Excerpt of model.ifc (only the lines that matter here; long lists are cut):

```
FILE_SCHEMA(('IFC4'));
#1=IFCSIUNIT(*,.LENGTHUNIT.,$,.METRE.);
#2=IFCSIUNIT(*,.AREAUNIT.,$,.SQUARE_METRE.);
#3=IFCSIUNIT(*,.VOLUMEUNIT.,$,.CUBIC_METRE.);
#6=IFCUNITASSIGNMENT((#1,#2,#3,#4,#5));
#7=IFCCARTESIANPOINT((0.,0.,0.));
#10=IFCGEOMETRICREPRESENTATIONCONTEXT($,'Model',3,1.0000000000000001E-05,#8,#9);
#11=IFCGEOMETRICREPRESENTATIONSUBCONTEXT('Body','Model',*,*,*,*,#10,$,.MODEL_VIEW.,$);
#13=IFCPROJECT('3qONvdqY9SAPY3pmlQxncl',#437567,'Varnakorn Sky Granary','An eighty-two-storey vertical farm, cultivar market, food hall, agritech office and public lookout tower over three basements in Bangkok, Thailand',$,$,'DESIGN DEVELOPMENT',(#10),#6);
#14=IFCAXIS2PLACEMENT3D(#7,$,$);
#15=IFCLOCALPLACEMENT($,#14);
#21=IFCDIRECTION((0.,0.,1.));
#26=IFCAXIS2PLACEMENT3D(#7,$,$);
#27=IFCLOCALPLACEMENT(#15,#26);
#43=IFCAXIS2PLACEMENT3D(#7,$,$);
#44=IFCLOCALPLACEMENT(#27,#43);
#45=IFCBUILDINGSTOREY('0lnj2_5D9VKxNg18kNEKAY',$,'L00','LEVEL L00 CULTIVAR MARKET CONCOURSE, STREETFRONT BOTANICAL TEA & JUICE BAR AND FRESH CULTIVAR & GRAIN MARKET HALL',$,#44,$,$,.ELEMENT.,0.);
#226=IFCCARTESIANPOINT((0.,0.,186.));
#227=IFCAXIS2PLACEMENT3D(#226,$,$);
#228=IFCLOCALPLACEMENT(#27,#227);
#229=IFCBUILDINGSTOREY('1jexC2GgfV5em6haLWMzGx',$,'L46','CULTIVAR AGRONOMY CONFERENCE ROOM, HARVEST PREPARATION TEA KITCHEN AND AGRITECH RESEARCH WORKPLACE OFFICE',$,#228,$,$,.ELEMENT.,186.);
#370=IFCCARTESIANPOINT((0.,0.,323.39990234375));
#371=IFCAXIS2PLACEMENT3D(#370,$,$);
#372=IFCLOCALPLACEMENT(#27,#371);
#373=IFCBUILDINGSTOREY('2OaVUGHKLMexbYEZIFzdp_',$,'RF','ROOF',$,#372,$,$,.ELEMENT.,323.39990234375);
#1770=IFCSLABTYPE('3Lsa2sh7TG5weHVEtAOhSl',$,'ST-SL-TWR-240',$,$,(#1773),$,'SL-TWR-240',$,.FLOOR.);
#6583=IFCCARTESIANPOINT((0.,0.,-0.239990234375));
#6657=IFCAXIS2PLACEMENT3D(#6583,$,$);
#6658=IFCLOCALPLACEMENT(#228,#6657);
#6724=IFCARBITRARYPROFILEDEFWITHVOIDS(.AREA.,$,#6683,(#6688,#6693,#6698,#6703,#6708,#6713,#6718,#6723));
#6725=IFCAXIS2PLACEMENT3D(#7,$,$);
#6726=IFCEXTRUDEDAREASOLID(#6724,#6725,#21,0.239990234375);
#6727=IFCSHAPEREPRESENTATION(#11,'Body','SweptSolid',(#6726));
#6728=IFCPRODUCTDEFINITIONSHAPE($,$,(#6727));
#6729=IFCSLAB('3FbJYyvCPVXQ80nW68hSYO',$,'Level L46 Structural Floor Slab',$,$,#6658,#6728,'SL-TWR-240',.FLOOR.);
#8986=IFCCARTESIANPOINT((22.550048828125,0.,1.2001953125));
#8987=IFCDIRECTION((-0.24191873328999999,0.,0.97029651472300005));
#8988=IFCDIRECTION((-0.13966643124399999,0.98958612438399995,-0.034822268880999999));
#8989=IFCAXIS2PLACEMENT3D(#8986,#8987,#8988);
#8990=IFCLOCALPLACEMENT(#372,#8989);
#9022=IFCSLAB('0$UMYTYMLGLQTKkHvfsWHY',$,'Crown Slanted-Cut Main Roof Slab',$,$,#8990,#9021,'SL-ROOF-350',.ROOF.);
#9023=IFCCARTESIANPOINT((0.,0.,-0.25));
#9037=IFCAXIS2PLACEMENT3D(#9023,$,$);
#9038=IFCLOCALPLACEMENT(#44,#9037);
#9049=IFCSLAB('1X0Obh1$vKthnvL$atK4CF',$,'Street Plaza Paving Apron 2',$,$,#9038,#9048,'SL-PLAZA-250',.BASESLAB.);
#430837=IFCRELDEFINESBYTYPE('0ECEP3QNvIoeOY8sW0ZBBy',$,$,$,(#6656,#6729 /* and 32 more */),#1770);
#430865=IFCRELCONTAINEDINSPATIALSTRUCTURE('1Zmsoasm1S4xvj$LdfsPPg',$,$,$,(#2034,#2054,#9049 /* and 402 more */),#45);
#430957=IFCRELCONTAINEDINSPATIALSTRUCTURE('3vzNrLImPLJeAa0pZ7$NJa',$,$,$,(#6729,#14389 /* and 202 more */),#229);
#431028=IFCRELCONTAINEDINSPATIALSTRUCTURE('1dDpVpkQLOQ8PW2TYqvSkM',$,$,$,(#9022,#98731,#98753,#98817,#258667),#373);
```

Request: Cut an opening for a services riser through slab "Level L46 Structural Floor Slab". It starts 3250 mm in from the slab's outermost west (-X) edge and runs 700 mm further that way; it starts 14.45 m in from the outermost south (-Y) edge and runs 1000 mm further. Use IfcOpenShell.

```python
import numpy as np
import ifcopenshell
import ifcopenshell.api.feature
import ifcopenshell.api.geometry
import ifcopenshell.api.root
import ifcopenshell.geom
import ifcopenshell.util.placement
import ifcopenshell.util.representation
import ifcopenshell.util.shape
import ifcopenshell.util.unit

model = ifcopenshell.open("model.ifc")
unit_scale = ifcopenshell.util.unit.calculate_unit_scale(model)
settings = ifcopenshell.geom.settings()


def volume(element):
    """Net volume in cubic metres, openings subtracted."""
    shape = ifcopenshell.geom.create_shape(settings, element)
    return ifcopenshell.util.shape.get_volume(shape.geometry)


slab = model.by_guid("3FbJYyvCPVXQ80nW68hSYO")
before = volume(slab)

# Extent in the slab's own axes, in metres. The edges named are its -X and -Y sides.
slab_shape = ifcopenshell.geom.create_shape(settings, slab)
vertices = ifcopenshell.util.shape.get_vertices(slab_shape.geometry)
x_min, y_min, bottom = vertices.min(axis=0)
top = vertices[:, 2].max()

opening = ifcopenshell.api.root.create_entity(model, ifc_class="IfcOpeningElement", name="Services riser opening", predefined_type="OPENING")
context = ifcopenshell.util.representation.get_context(model, "Model", "Body", "MODEL_VIEW")
width, depth = 0.7, 1
outline = [(0.0, 0.0), (width, 0.0), (width, depth), (0.0, depth), (0.0, 0.0)]
# Overshoot both faces by 50 mm so the cut is clean.
shape = ifcopenshell.api.geometry.add_slab_representation(
    model, context=context, depth=top - bottom + 0.1, polyline=outline
)
ifcopenshell.api.geometry.assign_representation(model, product=opening, representation=shape)

matrix = ifcopenshell.util.placement.get_local_placement(slab.ObjectPlacement)
matrix[:, 3] = matrix @ np.append(np.array([x_min + 3.25, y_min + 14.45, bottom - 0.05]) / unit_scale, 1.0)
ifcopenshell.api.geometry.edit_object_placement(model, product=opening, matrix=matrix, is_si=False)
ifcopenshell.api.feature.add_feature(model, feature=opening, element=slab)

after = volume(slab)

print(f"slab volume {before:.3f} -> {after:.3f} m3")

model.write("model_updated.ifc")
```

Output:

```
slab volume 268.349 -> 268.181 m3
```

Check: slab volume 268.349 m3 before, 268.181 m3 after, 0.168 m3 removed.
